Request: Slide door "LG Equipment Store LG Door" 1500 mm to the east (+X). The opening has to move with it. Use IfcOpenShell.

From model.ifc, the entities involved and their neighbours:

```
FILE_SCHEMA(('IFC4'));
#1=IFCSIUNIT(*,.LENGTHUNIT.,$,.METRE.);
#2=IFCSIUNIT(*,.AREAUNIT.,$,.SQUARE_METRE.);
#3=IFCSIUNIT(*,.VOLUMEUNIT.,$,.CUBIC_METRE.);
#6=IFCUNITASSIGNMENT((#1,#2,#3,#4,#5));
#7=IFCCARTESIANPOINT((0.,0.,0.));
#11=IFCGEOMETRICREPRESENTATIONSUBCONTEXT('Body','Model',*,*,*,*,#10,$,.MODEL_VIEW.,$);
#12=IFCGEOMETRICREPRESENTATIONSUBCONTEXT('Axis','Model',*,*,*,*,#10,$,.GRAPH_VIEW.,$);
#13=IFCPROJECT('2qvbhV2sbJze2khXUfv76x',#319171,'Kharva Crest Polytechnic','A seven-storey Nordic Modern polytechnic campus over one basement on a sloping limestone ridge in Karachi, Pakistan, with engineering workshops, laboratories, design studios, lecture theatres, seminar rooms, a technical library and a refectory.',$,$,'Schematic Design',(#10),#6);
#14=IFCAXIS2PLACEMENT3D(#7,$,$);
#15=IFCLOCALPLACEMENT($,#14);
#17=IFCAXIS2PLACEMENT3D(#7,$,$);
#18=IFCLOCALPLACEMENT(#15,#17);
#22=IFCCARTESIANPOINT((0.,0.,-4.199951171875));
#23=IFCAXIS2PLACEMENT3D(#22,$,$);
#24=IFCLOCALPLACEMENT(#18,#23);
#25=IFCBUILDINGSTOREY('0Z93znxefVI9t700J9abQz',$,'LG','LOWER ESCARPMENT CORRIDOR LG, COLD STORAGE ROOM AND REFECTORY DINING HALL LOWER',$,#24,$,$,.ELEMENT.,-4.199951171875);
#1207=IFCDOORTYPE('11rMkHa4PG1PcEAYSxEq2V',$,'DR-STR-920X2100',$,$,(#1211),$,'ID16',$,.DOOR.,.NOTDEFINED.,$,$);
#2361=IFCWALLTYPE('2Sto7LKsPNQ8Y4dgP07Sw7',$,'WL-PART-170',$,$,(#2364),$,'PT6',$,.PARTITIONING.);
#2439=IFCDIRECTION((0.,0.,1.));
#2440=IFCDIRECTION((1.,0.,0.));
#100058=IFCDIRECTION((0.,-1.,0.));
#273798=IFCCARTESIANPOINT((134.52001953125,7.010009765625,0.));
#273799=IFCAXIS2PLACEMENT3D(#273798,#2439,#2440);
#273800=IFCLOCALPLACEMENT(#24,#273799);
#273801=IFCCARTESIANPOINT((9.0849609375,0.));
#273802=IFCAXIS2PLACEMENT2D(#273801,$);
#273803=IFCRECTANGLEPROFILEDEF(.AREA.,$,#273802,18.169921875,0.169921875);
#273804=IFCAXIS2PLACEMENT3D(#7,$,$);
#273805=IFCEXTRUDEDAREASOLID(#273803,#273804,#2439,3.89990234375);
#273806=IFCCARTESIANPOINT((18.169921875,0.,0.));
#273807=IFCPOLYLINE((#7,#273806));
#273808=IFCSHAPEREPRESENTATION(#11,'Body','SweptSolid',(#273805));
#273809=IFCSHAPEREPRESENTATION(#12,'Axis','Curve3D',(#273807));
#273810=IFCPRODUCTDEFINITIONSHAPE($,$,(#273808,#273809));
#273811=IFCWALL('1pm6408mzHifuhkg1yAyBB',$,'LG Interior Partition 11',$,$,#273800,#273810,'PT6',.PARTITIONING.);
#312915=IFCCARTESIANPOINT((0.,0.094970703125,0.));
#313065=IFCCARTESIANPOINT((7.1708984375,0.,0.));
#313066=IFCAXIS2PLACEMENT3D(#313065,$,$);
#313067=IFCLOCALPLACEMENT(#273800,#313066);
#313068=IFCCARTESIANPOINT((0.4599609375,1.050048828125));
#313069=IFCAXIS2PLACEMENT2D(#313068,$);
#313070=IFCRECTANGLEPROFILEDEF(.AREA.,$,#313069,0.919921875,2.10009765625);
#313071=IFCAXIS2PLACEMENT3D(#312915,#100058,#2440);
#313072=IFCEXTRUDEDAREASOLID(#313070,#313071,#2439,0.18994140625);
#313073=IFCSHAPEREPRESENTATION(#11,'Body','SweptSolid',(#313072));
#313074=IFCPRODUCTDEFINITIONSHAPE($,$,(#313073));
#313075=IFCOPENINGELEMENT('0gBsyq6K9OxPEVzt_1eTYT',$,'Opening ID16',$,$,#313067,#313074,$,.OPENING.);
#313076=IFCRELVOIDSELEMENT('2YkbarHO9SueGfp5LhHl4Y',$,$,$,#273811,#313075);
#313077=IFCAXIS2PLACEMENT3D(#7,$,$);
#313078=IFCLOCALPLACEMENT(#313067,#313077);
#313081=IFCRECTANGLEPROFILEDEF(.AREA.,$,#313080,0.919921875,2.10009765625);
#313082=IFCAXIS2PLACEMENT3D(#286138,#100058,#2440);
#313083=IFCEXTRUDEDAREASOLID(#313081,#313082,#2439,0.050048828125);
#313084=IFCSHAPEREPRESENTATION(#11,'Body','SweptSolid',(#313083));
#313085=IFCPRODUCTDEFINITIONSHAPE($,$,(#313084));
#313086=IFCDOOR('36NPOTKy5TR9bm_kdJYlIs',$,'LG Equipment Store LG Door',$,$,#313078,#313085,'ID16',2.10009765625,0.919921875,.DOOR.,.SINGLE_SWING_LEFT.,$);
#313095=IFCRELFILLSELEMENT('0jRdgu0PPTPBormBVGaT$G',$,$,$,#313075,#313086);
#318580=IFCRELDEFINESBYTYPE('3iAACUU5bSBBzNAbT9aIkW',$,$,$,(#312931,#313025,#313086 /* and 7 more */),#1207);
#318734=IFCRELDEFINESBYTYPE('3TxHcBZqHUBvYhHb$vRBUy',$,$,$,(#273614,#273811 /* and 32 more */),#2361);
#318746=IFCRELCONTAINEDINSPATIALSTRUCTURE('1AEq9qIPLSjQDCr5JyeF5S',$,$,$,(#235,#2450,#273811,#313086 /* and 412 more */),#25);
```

```python
import ifcopenshell
import ifcopenshell.api.geometry
import ifcopenshell.util.placement
import ifcopenshell.util.unit

model = ifcopenshell.open("model.ifc")
unit_scale = ifcopenshell.util.unit.calculate_unit_scale(model)

door = model.by_guid("36NPOTKy5TR9bm_kdJYlIs")
opening = door.FillsVoids[0].RelatingOpeningElement
wall = opening.VoidsElements[0].RelatingBuildingElement

wall_matrix = ifcopenshell.util.placement.get_local_placement(wall.ObjectPlacement)
shift = wall_matrix[:3, 0] * 1.5 / unit_scale
before = ifcopenshell.util.placement.get_local_placement(door.ObjectPlacement)[:3, 3].copy()

# The door is placed relative to its opening, so it follows when the opening moves.
matrix = ifcopenshell.util.placement.get_local_placement(opening.ObjectPlacement)
matrix[:3, 3] += shift
ifcopenshell.api.geometry.edit_object_placement(
    model, product=opening, matrix=matrix, is_si=False, should_transform_children=True
)

after = ifcopenshell.util.placement.get_local_placement(door.ObjectPlacement)[:3, 3]
print("door moved by", (after - before).round(3) + 0.0)

model.write("model_updated.ifc")
```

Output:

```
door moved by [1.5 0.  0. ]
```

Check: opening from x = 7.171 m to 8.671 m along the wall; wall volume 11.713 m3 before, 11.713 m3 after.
